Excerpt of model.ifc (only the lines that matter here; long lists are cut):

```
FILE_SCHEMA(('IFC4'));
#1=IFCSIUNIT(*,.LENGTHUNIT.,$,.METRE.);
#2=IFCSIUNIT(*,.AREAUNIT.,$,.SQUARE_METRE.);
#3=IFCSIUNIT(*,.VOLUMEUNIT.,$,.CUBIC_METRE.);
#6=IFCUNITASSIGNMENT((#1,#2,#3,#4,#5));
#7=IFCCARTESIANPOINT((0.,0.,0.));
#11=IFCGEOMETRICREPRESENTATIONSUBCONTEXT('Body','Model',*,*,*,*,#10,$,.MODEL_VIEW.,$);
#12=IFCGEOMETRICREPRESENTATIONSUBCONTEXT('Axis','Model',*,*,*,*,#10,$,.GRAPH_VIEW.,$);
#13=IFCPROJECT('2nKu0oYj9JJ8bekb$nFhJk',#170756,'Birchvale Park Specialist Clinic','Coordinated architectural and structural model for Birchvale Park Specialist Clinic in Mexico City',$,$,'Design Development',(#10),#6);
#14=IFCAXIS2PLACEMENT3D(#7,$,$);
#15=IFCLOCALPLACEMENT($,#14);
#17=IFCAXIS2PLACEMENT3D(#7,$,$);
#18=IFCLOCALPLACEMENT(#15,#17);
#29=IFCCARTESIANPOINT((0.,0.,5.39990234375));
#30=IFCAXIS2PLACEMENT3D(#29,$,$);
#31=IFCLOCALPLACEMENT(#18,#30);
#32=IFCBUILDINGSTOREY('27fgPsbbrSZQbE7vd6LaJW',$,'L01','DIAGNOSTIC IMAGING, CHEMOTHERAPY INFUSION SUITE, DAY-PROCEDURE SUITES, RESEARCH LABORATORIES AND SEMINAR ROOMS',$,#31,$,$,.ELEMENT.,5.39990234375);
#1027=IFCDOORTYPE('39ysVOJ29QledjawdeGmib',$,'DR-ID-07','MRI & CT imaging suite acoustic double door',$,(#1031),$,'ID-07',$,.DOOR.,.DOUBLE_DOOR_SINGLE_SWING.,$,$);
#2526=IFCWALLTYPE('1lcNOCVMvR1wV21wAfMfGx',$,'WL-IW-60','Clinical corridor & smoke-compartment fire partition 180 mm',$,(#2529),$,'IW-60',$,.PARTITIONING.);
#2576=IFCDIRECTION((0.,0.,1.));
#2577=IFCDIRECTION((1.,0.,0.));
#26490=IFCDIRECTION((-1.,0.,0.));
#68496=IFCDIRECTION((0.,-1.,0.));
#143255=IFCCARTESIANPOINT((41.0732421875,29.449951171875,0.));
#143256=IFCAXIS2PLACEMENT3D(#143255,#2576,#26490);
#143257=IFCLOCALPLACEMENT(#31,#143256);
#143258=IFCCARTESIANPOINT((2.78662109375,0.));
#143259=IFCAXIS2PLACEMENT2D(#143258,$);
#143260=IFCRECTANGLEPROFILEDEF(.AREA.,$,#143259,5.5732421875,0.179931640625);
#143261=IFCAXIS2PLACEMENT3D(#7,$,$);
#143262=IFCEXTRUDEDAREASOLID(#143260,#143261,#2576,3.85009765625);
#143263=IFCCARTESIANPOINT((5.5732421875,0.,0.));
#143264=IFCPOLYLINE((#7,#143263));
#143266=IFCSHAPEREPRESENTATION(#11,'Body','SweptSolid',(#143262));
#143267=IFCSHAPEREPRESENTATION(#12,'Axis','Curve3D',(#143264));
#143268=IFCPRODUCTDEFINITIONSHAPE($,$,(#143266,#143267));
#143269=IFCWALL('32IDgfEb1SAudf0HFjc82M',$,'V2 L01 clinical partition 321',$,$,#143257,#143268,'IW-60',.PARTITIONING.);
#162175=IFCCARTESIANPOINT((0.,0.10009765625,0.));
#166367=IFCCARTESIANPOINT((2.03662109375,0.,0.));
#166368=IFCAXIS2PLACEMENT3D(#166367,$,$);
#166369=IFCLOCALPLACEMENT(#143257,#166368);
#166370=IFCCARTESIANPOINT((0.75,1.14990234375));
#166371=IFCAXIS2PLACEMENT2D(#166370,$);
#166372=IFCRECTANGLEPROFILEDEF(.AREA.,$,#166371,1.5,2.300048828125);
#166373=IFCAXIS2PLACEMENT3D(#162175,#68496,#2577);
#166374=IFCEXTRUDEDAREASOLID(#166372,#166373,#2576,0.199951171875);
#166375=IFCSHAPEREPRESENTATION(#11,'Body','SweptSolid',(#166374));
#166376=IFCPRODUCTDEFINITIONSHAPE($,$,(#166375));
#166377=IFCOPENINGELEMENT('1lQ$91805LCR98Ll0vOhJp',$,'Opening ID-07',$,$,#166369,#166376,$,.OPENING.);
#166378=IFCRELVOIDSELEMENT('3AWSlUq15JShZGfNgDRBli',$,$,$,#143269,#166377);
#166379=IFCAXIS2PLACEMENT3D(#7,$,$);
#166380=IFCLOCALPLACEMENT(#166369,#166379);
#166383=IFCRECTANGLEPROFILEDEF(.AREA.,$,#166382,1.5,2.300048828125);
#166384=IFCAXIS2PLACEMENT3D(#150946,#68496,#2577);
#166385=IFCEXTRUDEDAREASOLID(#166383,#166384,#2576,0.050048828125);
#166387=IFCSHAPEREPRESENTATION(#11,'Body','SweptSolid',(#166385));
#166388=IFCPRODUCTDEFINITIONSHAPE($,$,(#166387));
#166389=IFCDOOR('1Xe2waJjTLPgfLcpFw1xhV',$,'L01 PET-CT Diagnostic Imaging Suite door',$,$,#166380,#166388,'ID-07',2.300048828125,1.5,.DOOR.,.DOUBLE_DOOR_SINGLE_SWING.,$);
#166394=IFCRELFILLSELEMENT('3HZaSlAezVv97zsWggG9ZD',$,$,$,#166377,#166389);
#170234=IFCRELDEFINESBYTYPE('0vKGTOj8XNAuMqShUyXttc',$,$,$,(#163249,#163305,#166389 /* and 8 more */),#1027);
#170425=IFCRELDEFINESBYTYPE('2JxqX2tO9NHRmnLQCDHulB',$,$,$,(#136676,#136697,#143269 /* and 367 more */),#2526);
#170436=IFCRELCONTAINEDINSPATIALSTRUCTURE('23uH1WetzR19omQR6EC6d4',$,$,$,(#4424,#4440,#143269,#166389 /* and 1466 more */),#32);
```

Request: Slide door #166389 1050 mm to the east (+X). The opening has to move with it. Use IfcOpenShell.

```python
import ifcopenshell
import ifcopenshell.api.geometry
import ifcopenshell.util.placement
import ifcopenshell.util.unit

model = ifcopenshell.open("model.ifc")
unit_scale = ifcopenshell.util.unit.calculate_unit_scale(model)

door = model.by_guid("1Xe2waJjTLPgfLcpFw1xhV")
opening = door.FillsVoids[0].RelatingOpeningElement
wall = opening.VoidsElements[0].RelatingBuildingElement

wall_matrix = ifcopenshell.util.placement.get_local_placement(wall.ObjectPlacement)
shift = wall_matrix[:3, 0] * -1.05 / unit_scale
before = ifcopenshell.util.placement.get_local_placement(door.ObjectPlacement)[:3, 3].copy()

# The door is placed relative to its opening, so it follows when the opening moves.
matrix = ifcopenshell.util.placement.get_local_placement(opening.ObjectPlacement)
matrix[:3, 3] += shift
ifcopenshell.api.geometry.edit_object_placement(
    model, product=opening, matrix=matrix, is_si=False, should_transform_children=True
)

after = ifcopenshell.util.placement.get_local_placement(door.ObjectPlacement)[:3, 3]
print("door moved by", (after - before).round(3) + 0.0)

model.write("model_v2.ifc")
```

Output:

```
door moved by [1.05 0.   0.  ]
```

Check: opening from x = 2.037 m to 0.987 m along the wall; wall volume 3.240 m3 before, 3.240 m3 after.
